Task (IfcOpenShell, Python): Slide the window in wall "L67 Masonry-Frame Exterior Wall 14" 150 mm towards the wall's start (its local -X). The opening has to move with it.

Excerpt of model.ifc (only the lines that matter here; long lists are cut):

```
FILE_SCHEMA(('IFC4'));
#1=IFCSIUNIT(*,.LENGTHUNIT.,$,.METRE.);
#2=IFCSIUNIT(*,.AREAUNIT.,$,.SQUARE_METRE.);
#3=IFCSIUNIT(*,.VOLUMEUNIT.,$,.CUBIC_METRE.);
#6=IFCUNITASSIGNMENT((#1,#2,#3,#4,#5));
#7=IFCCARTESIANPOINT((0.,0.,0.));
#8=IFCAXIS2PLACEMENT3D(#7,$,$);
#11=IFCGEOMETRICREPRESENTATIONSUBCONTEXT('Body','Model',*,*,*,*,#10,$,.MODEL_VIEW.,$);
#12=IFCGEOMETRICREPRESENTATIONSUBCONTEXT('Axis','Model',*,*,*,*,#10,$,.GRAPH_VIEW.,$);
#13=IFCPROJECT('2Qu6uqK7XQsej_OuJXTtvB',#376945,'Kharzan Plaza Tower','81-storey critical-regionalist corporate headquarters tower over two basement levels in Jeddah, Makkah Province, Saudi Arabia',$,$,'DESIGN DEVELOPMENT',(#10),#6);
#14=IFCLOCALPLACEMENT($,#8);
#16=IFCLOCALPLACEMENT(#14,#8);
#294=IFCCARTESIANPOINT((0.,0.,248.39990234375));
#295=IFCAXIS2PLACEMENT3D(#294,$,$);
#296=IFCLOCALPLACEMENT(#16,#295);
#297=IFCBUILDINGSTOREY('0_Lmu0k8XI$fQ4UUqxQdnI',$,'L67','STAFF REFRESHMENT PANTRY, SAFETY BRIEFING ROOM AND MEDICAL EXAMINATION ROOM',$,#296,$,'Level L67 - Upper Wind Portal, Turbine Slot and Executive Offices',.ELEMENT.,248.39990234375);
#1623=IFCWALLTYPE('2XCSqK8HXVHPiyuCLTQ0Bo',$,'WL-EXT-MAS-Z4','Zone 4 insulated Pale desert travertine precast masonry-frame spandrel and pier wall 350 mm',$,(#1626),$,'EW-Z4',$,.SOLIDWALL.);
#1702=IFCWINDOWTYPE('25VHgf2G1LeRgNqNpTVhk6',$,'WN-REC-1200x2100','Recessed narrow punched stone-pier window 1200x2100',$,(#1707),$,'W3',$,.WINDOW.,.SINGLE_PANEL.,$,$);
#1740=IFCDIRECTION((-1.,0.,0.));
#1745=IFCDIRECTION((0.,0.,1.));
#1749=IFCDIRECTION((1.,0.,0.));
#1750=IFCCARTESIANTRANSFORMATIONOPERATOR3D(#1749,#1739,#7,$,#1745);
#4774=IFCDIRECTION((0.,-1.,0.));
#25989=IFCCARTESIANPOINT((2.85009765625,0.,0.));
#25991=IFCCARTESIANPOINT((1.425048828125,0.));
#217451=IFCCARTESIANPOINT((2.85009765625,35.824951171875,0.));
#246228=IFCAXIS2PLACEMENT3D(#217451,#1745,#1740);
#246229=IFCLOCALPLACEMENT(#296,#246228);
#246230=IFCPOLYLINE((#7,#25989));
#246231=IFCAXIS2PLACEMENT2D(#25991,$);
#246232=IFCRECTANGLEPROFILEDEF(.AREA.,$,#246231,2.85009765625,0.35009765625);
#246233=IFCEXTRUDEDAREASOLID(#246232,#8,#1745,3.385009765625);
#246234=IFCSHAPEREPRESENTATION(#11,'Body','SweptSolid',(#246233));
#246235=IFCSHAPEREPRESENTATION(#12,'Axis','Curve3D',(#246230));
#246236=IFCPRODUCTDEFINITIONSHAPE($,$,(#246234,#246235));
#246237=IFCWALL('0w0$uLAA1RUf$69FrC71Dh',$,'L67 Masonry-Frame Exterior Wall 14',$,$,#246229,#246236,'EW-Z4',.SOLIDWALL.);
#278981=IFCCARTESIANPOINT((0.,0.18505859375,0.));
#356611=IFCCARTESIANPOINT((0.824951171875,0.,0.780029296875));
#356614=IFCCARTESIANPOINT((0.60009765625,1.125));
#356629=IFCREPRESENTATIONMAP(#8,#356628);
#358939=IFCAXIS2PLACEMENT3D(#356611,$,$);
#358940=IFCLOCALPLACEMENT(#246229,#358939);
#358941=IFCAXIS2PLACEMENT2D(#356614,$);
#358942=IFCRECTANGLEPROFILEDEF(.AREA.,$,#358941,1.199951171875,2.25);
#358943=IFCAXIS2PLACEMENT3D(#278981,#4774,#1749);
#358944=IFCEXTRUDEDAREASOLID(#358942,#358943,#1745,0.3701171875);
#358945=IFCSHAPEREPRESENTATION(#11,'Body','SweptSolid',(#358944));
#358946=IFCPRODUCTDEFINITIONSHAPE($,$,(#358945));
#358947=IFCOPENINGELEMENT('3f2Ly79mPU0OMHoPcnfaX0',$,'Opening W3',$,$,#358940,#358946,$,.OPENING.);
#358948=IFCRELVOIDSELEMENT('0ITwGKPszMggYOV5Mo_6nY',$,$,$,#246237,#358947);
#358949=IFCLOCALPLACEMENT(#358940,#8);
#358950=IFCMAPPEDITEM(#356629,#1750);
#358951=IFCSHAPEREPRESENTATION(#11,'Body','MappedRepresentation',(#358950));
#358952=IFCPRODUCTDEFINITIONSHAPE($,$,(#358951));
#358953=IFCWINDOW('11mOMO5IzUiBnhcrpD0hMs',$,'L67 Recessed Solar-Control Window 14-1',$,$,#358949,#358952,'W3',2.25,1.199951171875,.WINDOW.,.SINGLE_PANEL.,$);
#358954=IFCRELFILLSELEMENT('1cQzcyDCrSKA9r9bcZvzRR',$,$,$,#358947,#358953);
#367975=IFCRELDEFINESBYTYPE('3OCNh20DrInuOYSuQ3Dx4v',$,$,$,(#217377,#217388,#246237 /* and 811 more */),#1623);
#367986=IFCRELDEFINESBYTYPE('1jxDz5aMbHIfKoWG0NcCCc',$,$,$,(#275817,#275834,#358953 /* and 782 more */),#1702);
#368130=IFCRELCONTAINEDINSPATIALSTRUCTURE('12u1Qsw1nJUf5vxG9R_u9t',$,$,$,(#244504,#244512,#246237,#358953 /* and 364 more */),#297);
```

```python
import ifcopenshell
import ifcopenshell.api.geometry
import ifcopenshell.util.placement

model = ifcopenshell.open("model.ifc")

window = model.by_guid("11mOMO5IzUiBnhcrpD0hMs")
opening = window.FillsVoids[0].RelatingOpeningElement
wall = opening.VoidsElements[0].RelatingBuildingElement

wall_matrix = ifcopenshell.util.placement.get_local_placement(wall.ObjectPlacement)
shift = wall_matrix[:3, 0] * -0.15
before = ifcopenshell.util.placement.get_local_placement(window.ObjectPlacement)[:3, 3].copy()

# The window is placed relative to its opening, so it follows when the opening moves.
matrix = ifcopenshell.util.placement.get_local_placement(opening.ObjectPlacement)
matrix[:3, 3] += shift
ifcopenshell.api.geometry.edit_object_placement(
    model, product=opening, matrix=matrix, is_si=False, should_transform_children=True
)

after = ifcopenshell.util.placement.get_local_placement(window.ObjectPlacement)[:3, 3]
print("window moved by", (after - before).round(3) + 0.0)

model.write("model-out.ifc")
```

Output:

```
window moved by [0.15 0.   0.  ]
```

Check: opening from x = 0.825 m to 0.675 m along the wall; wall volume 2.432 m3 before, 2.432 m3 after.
